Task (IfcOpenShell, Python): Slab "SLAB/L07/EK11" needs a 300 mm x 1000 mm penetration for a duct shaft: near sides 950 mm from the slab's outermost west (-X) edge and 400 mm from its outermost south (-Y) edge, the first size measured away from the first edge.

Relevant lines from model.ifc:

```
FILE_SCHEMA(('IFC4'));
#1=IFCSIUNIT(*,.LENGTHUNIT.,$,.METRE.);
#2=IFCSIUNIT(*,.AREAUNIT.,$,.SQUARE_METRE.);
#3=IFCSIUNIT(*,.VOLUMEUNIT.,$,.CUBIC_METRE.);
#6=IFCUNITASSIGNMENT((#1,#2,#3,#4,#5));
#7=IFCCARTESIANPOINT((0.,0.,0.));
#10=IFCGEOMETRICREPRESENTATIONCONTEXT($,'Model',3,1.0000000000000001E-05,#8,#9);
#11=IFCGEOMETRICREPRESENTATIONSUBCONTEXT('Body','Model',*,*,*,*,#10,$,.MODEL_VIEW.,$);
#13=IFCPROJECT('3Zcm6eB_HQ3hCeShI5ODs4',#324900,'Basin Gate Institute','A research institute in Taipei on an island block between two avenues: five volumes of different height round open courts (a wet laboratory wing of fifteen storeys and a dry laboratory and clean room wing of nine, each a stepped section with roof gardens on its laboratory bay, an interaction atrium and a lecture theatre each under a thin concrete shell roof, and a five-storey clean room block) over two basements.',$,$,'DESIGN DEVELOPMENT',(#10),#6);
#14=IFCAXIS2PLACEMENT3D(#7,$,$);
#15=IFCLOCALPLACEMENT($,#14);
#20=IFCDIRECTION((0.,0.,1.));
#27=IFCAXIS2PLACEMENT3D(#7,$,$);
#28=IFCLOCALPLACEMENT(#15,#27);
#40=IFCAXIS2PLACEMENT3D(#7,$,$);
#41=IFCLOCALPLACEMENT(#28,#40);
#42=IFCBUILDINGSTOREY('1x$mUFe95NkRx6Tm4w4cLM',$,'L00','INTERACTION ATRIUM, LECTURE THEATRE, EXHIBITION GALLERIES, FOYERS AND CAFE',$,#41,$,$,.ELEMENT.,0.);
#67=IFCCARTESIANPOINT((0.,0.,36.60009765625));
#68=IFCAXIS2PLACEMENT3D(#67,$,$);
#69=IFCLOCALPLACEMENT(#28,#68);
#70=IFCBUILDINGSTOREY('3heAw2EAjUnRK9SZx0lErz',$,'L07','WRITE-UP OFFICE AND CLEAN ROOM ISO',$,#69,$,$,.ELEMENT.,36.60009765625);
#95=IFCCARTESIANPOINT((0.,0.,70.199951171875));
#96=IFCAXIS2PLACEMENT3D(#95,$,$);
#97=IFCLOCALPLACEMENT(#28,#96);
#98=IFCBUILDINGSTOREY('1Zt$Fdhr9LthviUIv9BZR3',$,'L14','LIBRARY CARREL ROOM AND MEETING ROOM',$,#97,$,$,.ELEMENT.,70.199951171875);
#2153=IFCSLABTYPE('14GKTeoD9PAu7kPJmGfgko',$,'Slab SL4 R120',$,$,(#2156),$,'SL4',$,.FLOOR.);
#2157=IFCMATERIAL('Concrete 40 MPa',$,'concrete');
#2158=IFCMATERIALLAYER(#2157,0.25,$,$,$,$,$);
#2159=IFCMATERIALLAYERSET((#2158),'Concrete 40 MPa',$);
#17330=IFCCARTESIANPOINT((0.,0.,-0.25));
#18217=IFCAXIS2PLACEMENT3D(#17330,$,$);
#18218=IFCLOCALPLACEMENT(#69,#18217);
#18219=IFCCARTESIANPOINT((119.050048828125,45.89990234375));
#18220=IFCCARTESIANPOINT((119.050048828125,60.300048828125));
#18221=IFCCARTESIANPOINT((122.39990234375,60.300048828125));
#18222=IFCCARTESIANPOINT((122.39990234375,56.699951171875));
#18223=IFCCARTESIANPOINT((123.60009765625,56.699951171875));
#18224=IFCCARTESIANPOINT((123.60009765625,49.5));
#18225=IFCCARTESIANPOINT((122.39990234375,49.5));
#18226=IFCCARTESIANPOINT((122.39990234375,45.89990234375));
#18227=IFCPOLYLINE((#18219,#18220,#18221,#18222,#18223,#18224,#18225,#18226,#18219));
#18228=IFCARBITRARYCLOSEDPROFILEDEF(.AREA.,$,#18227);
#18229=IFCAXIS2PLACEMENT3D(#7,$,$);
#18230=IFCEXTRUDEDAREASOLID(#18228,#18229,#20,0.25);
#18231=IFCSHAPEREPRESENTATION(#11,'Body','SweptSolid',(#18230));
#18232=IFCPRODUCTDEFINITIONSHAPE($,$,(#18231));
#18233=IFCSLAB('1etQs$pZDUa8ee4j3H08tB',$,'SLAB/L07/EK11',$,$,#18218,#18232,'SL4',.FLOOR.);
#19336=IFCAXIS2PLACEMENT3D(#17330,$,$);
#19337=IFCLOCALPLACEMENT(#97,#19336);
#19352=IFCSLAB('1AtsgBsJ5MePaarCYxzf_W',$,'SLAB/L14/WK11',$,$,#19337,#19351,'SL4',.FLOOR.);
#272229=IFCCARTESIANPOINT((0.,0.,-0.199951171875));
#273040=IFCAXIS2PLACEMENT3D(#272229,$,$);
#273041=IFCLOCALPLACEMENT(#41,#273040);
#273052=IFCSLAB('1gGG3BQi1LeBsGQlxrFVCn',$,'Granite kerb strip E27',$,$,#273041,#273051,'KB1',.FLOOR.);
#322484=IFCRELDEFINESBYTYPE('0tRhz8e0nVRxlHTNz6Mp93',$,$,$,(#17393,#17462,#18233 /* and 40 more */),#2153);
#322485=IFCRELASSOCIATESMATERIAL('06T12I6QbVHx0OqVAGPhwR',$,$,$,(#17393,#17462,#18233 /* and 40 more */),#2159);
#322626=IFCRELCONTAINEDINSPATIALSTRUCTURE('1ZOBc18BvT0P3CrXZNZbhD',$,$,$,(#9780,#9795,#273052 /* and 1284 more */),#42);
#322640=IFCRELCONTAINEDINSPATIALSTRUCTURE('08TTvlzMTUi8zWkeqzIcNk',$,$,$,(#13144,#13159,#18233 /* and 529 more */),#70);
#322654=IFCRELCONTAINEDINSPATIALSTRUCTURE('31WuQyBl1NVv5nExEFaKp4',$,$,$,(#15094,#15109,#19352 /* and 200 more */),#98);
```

```python
import numpy as np
import ifcopenshell
import ifcopenshell.api.feature
import ifcopenshell.api.geometry
import ifcopenshell.api.root
import ifcopenshell.geom
import ifcopenshell.util.placement
import ifcopenshell.util.representation
import ifcopenshell.util.shape
import ifcopenshell.util.unit

model = ifcopenshell.open("model.ifc")
unit_scale = ifcopenshell.util.unit.calculate_unit_scale(model)
settings = ifcopenshell.geom.settings()


def volume(element):
    """Net volume in cubic metres, openings subtracted."""
    shape = ifcopenshell.geom.create_shape(settings, element)
    return ifcopenshell.util.shape.get_volume(shape.geometry)


slab = model.by_guid("1etQs$pZDUa8ee4j3H08tB")
before = volume(slab)

# Extent in the slab's own axes, in metres. The edges named are its -X and -Y sides.
slab_shape = ifcopenshell.geom.create_shape(settings, slab)
vertices = ifcopenshell.util.shape.get_vertices(slab_shape.geometry)
x_min, y_min, bottom = vertices.min(axis=0)
top = vertices[:, 2].max()

opening = ifcopenshell.api.root.create_entity(model, ifc_class="IfcOpeningElement", name="Duct shaft opening", predefined_type="OPENING")
context = ifcopenshell.util.representation.get_context(model, "Model", "Body", "MODEL_VIEW")
width, depth = 0.3, 1
outline = [(0.0, 0.0), (width, 0.0), (width, depth), (0.0, depth), (0.0, 0.0)]
# Overshoot both faces by 50 mm so the cut is clean.
shape = ifcopenshell.api.geometry.add_slab_representation(
    model, context=context, depth=top - bottom + 0.1, polyline=outline
)
ifcopenshell.api.geometry.assign_representation(model, product=opening, representation=shape)

matrix = ifcopenshell.util.placement.get_local_placement(slab.ObjectPlacement)
matrix[:, 3] = matrix @ np.append(np.array([x_min + 0.95, y_min + 0.4, bottom - 0.05]) / unit_scale, 1.0)
ifcopenshell.api.geometry.edit_object_placement(model, product=opening, matrix=matrix, is_si=False)
ifcopenshell.api.feature.add_feature(model, feature=opening, element=slab)

after = volume(slab)

print(f"slab volume {before:.3f} -> {after:.3f} m3")

model.write("model_edited.ifc")
```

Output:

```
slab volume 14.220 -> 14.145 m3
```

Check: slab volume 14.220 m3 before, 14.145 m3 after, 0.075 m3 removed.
